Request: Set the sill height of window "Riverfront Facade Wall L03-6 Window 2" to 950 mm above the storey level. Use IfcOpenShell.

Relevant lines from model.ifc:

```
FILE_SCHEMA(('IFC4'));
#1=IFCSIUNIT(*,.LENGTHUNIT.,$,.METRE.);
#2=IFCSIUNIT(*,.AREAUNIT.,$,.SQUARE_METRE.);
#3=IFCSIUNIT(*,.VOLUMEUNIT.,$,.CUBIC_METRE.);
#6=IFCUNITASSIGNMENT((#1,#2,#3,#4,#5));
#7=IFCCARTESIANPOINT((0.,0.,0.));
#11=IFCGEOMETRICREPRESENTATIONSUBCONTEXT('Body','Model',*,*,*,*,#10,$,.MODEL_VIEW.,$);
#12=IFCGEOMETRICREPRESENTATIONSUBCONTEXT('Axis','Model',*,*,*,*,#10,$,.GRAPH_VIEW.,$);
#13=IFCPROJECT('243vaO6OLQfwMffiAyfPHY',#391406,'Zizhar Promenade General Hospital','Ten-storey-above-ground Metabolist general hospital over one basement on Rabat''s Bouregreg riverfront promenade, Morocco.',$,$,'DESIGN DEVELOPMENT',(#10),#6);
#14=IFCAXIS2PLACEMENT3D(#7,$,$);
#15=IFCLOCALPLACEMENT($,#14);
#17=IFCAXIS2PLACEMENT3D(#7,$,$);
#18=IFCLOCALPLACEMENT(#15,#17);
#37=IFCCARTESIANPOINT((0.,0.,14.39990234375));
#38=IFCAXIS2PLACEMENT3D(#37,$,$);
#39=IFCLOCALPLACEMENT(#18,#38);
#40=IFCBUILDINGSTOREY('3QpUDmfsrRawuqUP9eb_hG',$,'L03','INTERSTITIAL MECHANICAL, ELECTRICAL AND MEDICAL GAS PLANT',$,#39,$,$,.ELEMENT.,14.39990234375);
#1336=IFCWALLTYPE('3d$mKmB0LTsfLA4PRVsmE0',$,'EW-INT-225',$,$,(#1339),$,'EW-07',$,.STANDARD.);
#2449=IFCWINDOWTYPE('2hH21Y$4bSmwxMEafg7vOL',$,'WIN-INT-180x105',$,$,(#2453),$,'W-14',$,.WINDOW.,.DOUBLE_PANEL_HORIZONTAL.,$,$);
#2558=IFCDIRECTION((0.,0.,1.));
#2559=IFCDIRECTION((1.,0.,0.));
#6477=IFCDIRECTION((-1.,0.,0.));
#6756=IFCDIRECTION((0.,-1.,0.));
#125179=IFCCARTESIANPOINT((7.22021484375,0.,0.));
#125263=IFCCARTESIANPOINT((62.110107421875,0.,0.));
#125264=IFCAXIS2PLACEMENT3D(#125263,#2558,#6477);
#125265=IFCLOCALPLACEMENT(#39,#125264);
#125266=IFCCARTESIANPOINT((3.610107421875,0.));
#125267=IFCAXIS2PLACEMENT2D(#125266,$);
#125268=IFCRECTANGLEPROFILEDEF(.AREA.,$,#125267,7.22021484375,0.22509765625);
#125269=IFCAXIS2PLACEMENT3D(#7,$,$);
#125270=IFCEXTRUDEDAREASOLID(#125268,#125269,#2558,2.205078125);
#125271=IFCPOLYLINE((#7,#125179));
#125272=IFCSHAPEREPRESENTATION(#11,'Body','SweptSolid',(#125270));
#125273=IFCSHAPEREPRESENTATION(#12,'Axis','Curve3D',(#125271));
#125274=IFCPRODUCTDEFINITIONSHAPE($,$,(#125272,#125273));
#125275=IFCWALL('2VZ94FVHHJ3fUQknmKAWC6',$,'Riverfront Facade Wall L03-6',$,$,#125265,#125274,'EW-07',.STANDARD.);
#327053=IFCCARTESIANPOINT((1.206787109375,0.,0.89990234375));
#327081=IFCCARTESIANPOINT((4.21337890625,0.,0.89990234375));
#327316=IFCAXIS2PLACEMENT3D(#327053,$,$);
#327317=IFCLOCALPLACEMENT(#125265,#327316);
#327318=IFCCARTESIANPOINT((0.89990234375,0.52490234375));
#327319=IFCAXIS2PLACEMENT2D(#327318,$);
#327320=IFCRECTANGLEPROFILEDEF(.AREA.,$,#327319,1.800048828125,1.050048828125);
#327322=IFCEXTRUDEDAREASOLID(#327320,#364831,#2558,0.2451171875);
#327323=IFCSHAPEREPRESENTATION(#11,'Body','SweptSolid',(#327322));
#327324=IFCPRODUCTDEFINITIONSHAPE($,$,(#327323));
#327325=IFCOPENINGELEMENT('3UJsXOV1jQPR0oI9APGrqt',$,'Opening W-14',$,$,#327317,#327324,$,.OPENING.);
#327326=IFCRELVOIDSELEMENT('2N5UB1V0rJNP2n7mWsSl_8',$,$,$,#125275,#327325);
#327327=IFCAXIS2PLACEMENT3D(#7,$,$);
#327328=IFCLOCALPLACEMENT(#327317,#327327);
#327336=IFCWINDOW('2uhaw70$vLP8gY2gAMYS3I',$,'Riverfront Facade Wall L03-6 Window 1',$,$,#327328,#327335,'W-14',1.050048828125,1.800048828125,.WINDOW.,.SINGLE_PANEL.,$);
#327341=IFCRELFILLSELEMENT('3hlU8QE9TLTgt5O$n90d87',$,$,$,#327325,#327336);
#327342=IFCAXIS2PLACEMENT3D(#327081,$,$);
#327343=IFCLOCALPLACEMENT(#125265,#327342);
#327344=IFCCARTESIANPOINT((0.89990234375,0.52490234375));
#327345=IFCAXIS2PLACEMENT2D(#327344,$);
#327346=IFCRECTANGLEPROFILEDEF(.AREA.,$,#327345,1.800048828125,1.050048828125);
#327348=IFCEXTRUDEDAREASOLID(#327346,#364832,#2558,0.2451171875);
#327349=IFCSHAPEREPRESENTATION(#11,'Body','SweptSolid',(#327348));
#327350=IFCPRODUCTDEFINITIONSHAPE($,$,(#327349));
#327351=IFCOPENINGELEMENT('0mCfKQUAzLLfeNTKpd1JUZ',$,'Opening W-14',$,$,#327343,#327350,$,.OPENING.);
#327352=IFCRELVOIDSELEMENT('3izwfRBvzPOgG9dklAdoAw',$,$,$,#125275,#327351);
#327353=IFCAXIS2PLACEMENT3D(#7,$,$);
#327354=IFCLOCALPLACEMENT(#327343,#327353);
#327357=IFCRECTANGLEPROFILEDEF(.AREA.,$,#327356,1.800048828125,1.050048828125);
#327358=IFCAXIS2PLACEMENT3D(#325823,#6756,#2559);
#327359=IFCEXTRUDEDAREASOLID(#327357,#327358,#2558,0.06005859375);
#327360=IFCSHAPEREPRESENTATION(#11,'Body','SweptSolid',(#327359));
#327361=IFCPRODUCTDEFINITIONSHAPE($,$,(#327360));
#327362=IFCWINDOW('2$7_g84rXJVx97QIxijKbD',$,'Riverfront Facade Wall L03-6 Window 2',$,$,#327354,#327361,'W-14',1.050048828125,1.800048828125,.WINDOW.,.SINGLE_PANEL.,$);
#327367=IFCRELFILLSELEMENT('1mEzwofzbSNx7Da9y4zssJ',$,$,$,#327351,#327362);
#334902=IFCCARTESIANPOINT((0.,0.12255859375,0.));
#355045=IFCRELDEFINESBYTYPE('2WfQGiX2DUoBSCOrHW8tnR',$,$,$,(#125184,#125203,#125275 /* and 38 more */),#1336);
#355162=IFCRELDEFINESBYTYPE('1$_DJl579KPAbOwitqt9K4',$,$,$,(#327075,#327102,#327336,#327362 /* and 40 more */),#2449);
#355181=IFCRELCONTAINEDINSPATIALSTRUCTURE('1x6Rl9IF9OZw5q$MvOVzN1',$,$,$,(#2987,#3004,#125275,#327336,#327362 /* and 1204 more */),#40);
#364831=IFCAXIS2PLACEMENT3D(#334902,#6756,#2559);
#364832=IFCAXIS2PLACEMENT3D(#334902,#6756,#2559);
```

```python
import numpy as np
import ifcopenshell
import ifcopenshell.api.geometry
import ifcopenshell.geom
import ifcopenshell.util.element
import ifcopenshell.util.placement
import ifcopenshell.util.shape
import ifcopenshell.util.unit

model = ifcopenshell.open("model.ifc")
unit_scale = ifcopenshell.util.unit.calculate_unit_scale(model)

window = model.by_guid("2$7_g84rXJVx97QIxijKbD")
opening = window.FillsVoids[0].RelatingOpeningElement
storey = ifcopenshell.util.element.get_container(window, ifc_class="IfcBuildingStorey")
level = ifcopenshell.util.placement.get_local_placement(storey.ObjectPlacement)[2, 3]

# The opening's origin need not be at the sill, so measure its lowest point.
shape = ifcopenshell.geom.create_shape(ifcopenshell.geom.settings(), opening)
bottom = ifcopenshell.util.shape.get_shape_bottom_elevation(shape, shape.geometry) / unit_scale
dz = level + 0.95 / unit_scale - bottom

shift = np.array([0.0, 0.0, dz])
# The window is placed relative to its opening, so it follows when the opening moves.
matrix = ifcopenshell.util.placement.get_local_placement(opening.ObjectPlacement)
matrix[:3, 3] += shift
ifcopenshell.api.geometry.edit_object_placement(
    model, product=opening, matrix=matrix, is_si=False, should_transform_children=True
)

print(f"moved by {dz * unit_scale:+.3f} m")

model.write("model_edited.ifc")
```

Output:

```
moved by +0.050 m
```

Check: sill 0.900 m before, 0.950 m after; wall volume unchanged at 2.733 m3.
